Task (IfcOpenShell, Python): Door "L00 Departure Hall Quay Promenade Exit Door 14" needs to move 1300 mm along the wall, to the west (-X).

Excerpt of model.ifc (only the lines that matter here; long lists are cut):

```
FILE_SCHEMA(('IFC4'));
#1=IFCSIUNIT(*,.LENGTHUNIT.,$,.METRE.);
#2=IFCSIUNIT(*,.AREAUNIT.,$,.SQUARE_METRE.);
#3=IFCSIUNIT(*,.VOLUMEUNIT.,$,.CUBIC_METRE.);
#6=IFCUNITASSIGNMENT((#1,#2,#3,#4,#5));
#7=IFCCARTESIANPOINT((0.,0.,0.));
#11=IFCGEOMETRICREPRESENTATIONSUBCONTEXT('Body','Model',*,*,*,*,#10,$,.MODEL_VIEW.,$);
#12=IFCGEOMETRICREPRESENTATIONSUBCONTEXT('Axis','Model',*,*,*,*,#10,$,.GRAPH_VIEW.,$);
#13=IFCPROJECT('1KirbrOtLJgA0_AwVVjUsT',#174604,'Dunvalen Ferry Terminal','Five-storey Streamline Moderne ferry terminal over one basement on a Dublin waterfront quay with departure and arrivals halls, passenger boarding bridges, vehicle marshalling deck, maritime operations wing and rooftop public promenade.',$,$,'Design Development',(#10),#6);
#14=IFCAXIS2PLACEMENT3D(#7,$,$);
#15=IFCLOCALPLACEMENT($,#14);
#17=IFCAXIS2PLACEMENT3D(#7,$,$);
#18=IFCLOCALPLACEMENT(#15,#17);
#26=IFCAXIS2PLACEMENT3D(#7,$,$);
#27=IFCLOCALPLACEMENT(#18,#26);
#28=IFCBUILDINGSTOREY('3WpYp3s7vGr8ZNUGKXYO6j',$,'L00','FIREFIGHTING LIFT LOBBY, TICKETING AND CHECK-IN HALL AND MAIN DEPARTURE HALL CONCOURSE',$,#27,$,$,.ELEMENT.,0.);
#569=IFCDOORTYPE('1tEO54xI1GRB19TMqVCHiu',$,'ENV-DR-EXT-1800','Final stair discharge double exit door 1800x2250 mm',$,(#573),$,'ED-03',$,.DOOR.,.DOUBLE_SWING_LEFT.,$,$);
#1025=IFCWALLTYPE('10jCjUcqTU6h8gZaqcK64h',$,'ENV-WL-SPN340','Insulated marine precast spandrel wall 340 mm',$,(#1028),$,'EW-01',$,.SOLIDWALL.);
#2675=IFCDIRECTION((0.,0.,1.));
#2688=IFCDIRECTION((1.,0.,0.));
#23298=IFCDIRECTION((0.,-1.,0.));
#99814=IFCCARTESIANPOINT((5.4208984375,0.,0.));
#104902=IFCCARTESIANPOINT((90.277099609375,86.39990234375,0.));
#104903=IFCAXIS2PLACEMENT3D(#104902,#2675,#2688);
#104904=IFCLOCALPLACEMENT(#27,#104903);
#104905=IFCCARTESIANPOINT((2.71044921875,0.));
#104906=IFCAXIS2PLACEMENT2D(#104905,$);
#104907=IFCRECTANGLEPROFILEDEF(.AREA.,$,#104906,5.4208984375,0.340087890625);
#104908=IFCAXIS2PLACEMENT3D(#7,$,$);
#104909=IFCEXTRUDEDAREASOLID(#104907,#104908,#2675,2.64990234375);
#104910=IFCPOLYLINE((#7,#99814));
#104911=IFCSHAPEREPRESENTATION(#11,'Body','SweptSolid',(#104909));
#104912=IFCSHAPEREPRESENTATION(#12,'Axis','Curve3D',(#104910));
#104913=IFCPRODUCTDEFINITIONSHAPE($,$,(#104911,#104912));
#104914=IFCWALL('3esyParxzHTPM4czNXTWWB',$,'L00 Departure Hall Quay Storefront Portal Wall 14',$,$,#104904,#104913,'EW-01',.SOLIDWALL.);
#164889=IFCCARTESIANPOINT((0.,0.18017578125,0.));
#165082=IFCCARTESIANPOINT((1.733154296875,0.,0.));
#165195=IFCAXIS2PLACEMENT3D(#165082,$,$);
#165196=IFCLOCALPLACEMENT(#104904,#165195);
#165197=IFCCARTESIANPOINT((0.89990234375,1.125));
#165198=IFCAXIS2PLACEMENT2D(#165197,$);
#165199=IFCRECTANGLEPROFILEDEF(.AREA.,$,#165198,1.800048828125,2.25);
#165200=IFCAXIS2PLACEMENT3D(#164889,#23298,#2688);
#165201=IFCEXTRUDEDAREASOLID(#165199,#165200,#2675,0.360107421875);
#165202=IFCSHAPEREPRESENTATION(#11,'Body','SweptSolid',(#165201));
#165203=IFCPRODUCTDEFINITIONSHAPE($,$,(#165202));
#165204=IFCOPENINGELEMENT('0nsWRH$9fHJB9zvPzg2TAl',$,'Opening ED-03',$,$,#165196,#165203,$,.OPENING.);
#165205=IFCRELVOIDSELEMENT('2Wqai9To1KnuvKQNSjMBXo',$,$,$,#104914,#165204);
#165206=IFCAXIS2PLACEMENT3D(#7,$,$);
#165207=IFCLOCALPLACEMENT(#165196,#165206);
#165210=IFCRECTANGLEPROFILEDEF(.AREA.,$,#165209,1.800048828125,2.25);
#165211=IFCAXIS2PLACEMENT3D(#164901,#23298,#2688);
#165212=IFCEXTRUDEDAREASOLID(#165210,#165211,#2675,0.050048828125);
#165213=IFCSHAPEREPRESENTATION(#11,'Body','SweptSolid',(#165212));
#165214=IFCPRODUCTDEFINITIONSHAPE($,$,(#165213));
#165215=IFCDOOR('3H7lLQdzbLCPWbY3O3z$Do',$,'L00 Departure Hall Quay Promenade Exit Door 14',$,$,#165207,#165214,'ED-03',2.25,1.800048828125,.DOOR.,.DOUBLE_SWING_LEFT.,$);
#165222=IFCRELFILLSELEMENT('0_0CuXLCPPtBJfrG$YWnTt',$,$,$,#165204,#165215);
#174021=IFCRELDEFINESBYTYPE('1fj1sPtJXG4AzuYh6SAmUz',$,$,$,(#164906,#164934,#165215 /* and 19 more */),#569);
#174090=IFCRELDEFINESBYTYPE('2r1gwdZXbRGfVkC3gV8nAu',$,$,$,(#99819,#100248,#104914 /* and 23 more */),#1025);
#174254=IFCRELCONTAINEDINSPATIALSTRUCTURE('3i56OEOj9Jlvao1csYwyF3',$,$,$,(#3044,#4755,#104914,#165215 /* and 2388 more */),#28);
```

```python
import ifcopenshell
import ifcopenshell.api.geometry
import ifcopenshell.util.placement
import ifcopenshell.util.unit

model = ifcopenshell.open("model.ifc")
unit_scale = ifcopenshell.util.unit.calculate_unit_scale(model)

door = model.by_guid("3H7lLQdzbLCPWbY3O3z$Do")
opening = door.FillsVoids[0].RelatingOpeningElement
wall = opening.VoidsElements[0].RelatingBuildingElement

wall_matrix = ifcopenshell.util.placement.get_local_placement(wall.ObjectPlacement)
shift = wall_matrix[:3, 0] * -1.3 / unit_scale
before = ifcopenshell.util.placement.get_local_placement(door.ObjectPlacement)[:3, 3].copy()

# The door is placed relative to its opening, so it follows when the opening moves.
matrix = ifcopenshell.util.placement.get_local_placement(opening.ObjectPlacement)
matrix[:3, 3] += shift
ifcopenshell.api.geometry.edit_object_placement(
    model, product=opening, matrix=matrix, is_si=False, should_transform_children=True
)

after = ifcopenshell.util.placement.get_local_placement(door.ObjectPlacement)[:3, 3]
print("door moved by", (after - before).round(3) + 0.0)

model.write("model_edited.ifc")
```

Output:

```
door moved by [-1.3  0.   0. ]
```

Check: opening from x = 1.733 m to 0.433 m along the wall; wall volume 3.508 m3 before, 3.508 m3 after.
